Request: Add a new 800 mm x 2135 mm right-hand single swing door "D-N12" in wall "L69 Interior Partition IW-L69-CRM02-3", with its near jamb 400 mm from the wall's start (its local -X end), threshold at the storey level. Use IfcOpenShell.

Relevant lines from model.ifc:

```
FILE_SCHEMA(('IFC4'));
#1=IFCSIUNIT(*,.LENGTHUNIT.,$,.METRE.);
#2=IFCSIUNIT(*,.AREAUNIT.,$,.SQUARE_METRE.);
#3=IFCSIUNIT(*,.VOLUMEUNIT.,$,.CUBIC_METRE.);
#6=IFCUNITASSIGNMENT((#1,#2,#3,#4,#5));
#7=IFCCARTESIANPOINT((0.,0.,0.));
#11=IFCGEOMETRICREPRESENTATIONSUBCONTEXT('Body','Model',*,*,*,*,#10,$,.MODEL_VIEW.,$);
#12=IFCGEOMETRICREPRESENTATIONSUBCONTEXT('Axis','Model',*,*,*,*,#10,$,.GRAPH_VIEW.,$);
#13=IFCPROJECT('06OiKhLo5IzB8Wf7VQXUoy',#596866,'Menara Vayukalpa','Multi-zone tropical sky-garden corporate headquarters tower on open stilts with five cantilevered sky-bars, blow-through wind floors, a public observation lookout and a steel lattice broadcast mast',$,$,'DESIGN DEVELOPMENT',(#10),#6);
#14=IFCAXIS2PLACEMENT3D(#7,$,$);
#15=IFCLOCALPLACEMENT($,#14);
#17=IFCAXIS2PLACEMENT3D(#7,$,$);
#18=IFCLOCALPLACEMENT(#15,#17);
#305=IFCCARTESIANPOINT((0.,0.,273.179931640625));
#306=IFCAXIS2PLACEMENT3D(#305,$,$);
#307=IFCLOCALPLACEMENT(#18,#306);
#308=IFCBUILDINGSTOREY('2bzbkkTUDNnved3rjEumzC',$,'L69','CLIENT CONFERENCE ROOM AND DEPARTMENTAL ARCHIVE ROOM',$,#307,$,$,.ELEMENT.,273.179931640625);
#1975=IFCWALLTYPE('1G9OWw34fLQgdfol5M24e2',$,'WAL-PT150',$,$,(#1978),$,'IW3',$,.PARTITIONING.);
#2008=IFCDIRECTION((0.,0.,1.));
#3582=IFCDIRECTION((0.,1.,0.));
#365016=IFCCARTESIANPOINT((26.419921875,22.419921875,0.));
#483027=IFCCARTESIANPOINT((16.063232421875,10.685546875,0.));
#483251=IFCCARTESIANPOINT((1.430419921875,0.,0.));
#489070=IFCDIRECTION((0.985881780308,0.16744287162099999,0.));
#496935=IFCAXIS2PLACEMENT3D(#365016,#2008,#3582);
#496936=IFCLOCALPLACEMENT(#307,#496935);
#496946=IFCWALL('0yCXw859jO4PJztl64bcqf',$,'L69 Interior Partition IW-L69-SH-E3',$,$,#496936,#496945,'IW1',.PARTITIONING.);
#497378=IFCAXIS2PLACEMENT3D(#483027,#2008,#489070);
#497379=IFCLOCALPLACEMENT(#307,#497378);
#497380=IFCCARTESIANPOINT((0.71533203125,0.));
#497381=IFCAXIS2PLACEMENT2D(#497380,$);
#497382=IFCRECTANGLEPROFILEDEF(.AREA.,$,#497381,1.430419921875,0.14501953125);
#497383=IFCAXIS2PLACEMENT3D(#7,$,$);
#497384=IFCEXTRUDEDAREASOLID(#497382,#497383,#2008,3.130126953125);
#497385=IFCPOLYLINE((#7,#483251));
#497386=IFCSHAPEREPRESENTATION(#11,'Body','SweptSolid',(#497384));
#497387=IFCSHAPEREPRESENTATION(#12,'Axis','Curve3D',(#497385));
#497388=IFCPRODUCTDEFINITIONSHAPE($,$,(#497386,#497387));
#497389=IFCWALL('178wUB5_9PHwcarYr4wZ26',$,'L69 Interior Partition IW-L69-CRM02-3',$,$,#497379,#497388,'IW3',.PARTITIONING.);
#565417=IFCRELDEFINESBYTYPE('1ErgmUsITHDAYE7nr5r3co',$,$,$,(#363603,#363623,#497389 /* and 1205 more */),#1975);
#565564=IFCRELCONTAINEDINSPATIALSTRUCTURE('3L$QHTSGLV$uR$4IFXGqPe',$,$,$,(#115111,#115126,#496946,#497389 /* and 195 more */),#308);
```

```python
import numpy as np
import ifcopenshell
import ifcopenshell.api.feature
import ifcopenshell.api.geometry
import ifcopenshell.api.root
import ifcopenshell.api.spatial
import ifcopenshell.geom
import ifcopenshell.util.element
import ifcopenshell.util.placement
import ifcopenshell.util.representation
import ifcopenshell.util.shape
import ifcopenshell.util.unit

model = ifcopenshell.open("model.ifc")
unit_scale = ifcopenshell.util.unit.calculate_unit_scale(model)
settings = ifcopenshell.geom.settings()


def volume(element):
    """Net volume in cubic metres, openings subtracted."""
    shape = ifcopenshell.geom.create_shape(settings, element)
    return ifcopenshell.util.shape.get_volume(shape.geometry)


wall = model.by_guid("178wUB5_9PHwcarYr4wZ26")
storey = ifcopenshell.util.element.get_container(wall, ifc_class="IfcBuildingStorey")
context = ifcopenshell.util.representation.get_context(model, "Model", "Body", "MODEL_VIEW")
before = volume(wall)

width, height, from_end, sill = 0.8, 2.135, 0.4, 0.0  # metres

# The wall runs along its own X axis, and the end named is its -X end.
wall_shape = ifcopenshell.geom.create_shape(settings, wall)
x, y, z = ifcopenshell.util.shape.get_vertices(wall_shape.geometry).T
start = x.min() + from_end
face, thickness = float(y.min()), float(y.max() - y.min())
wall_matrix = ifcopenshell.util.placement.get_local_placement(wall.ObjectPlacement)
level = ifcopenshell.util.placement.get_local_placement(storey.ObjectPlacement)[2, 3]


def in_wall(x, y):
    """Placement at x, y metres in the wall's axes, at sill height."""
    matrix = wall_matrix.copy()
    matrix[:, 3] = wall_matrix @ np.array([x / unit_scale, y / unit_scale, 0.0, 1.0])
    matrix[2, 3] = level + sill / unit_scale
    return matrix


# Opening: a box that overshoots both wall faces by 50 mm.
opening = ifcopenshell.api.root.create_entity(model, ifc_class="IfcOpeningElement", predefined_type="OPENING")
box = ifcopenshell.api.geometry.add_wall_representation(
    model, context=context, length=width, height=height, thickness=thickness + 0.1
)
ifcopenshell.api.geometry.assign_representation(model, product=opening, representation=box)
ifcopenshell.api.geometry.edit_object_placement(model, product=opening, matrix=in_wall(start, face - 0.05), is_si=False)
ifcopenshell.api.feature.add_feature(model, feature=opening, element=wall)

door = ifcopenshell.api.root.create_entity(model, ifc_class="IfcDoor", name="D-N12", predefined_type="DOOR")
door.OverallWidth, door.OverallHeight = width / unit_scale, height / unit_scale
door.OperationType = "SINGLE_SWING_RIGHT"
body = ifcopenshell.api.geometry.add_door_representation(
    model,
    context=context,
    overall_width=door.OverallWidth,
    overall_height=door.OverallHeight,
    operation_type="SINGLE_SWING_RIGHT",
    lining_properties={"LiningDepth": thickness / unit_scale, "ThresholdDepth": thickness / unit_scale},
)
ifcopenshell.api.geometry.assign_representation(model, product=door, representation=body)
ifcopenshell.api.spatial.assign_container(model, products=[door], relating_structure=storey)
ifcopenshell.api.feature.add_filling(model, opening=opening, element=door)

# The lining spans the wall, so the door starts at the wall face.
ifcopenshell.api.geometry.edit_object_placement(model, product=door, matrix=in_wall(start, face), is_si=False)

after = volume(wall)

print(f"wall volume {before:.3f} -> {after:.3f} m3")

model.write("model_v2.ifc")
```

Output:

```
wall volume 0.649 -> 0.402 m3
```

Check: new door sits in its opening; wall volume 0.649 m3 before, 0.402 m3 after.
